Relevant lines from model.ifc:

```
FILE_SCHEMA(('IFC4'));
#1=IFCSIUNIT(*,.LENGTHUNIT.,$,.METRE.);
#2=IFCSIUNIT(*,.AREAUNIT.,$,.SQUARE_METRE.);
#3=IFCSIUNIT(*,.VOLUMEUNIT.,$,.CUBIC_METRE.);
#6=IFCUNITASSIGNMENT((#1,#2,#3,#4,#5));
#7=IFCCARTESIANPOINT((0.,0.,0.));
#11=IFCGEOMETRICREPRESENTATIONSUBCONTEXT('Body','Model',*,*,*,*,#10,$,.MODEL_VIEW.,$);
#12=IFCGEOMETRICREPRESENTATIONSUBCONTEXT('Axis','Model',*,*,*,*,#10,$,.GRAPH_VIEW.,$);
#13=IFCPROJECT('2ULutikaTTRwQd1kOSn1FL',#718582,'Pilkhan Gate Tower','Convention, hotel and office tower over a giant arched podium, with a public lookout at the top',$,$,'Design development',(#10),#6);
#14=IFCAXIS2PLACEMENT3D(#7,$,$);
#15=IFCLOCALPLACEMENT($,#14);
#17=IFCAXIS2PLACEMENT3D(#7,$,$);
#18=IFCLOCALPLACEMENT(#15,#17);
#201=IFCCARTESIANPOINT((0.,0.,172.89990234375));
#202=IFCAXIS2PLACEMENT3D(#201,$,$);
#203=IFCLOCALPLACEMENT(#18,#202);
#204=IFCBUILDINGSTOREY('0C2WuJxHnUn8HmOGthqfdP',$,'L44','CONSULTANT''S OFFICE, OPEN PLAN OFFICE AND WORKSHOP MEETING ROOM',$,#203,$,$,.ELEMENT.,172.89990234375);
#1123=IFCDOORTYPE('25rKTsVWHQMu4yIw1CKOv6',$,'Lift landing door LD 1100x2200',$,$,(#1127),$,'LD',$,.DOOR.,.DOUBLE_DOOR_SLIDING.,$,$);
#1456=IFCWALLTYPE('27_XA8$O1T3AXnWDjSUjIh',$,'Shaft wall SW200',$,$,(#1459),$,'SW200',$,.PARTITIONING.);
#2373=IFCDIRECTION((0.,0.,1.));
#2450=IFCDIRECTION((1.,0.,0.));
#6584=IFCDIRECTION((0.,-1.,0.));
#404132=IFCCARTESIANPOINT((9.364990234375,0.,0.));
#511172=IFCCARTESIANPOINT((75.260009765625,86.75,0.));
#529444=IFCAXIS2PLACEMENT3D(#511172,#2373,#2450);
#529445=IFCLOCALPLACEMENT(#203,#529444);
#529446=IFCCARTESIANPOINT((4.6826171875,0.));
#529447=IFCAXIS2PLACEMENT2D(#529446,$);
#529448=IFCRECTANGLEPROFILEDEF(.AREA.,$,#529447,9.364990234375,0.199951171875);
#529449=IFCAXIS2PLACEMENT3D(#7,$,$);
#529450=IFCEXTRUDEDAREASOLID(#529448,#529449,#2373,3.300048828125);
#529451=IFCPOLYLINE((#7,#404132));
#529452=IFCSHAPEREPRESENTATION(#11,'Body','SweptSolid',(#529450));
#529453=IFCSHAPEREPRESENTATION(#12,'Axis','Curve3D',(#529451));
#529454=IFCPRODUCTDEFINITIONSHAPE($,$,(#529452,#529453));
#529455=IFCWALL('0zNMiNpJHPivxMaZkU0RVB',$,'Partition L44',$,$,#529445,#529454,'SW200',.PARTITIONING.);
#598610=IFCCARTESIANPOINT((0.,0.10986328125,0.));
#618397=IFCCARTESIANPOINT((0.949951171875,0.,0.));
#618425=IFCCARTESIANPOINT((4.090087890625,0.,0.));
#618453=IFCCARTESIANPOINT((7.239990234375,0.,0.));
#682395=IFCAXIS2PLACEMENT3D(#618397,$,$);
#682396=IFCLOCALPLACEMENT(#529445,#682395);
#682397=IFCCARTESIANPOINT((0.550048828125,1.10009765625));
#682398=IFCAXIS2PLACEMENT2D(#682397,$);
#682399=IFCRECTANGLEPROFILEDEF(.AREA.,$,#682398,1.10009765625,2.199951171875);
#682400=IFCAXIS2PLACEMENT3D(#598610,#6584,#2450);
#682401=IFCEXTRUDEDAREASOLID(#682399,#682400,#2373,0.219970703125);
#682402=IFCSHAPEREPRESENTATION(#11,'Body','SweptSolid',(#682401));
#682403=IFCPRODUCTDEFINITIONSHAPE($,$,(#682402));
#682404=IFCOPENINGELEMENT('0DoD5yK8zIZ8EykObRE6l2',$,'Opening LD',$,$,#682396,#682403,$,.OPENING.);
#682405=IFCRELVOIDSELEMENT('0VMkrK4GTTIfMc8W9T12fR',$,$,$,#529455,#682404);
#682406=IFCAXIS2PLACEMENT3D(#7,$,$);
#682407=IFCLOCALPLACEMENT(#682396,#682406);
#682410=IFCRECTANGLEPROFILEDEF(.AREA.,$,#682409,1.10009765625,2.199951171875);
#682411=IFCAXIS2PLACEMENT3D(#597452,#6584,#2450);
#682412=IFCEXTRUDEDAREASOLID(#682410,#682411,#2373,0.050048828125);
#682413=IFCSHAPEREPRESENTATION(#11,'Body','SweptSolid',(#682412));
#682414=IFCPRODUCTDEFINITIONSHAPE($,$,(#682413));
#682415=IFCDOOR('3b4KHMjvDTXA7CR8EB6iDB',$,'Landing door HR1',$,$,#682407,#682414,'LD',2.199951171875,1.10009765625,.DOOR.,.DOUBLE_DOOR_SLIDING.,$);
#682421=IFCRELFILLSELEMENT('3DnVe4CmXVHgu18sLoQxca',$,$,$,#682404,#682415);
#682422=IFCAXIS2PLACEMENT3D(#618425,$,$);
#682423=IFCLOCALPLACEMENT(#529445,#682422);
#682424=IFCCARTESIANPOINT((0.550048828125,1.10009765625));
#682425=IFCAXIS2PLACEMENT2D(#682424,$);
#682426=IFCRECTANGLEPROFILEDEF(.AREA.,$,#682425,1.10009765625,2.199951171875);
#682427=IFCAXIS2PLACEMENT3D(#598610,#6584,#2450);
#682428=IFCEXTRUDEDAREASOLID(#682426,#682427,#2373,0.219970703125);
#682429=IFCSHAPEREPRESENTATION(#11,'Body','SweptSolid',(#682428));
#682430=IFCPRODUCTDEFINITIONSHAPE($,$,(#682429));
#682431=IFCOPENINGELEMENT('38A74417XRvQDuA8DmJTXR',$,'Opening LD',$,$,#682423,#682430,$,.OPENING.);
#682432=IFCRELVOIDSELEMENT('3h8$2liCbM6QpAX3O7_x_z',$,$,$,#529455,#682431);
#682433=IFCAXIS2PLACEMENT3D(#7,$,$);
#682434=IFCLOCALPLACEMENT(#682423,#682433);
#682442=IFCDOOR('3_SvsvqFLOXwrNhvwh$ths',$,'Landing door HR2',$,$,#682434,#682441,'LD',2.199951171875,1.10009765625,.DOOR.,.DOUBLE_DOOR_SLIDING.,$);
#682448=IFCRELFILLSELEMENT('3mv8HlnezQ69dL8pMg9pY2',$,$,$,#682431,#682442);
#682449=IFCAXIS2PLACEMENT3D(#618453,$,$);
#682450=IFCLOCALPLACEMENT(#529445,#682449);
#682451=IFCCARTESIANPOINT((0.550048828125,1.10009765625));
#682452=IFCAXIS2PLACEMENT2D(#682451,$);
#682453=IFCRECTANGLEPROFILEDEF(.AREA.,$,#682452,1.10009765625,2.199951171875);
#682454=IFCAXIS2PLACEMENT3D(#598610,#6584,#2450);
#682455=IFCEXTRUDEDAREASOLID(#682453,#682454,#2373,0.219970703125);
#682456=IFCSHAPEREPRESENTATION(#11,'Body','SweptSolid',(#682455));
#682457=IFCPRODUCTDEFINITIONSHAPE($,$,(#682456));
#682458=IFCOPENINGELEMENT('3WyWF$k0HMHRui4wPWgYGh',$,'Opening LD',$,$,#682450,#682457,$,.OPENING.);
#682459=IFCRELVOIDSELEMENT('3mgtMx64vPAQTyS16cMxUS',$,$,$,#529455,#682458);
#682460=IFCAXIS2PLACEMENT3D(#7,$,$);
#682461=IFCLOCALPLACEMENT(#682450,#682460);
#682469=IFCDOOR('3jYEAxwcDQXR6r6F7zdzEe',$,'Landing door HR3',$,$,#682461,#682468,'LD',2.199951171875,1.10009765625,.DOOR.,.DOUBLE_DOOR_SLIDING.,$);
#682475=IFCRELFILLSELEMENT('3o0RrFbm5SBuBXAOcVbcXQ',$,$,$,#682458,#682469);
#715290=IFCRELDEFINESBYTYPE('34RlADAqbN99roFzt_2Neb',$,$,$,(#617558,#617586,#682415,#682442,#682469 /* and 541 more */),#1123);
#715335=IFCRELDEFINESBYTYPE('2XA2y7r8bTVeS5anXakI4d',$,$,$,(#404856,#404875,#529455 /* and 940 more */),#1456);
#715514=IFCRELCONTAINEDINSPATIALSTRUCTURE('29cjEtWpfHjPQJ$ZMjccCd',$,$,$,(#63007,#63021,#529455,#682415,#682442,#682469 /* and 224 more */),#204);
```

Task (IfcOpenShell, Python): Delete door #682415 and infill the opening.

```python
import ifcopenshell
import ifcopenshell.api.feature
import ifcopenshell.api.root
import ifcopenshell.geom
import ifcopenshell.util.shape

model = ifcopenshell.open("model.ifc")
settings = ifcopenshell.geom.settings()


def volume(element):
    """Net volume in cubic metres, openings subtracted."""
    shape = ifcopenshell.geom.create_shape(settings, element)
    return ifcopenshell.util.shape.get_volume(shape.geometry)


door = model.by_id(682415)
opening = door.FillsVoids[0].RelatingOpeningElement
wall = opening.VoidsElements[0].RelatingBuildingElement
before = volume(wall)

ifcopenshell.api.root.remove_product(model, product=door)
ifcopenshell.api.feature.remove_feature(model, feature=opening)

after = volume(wall)

print(f"wall volume {before:.3f} -> {after:.3f} m3")

model.write("model_updated.ifc")
```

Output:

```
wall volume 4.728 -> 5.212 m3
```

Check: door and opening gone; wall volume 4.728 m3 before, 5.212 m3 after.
